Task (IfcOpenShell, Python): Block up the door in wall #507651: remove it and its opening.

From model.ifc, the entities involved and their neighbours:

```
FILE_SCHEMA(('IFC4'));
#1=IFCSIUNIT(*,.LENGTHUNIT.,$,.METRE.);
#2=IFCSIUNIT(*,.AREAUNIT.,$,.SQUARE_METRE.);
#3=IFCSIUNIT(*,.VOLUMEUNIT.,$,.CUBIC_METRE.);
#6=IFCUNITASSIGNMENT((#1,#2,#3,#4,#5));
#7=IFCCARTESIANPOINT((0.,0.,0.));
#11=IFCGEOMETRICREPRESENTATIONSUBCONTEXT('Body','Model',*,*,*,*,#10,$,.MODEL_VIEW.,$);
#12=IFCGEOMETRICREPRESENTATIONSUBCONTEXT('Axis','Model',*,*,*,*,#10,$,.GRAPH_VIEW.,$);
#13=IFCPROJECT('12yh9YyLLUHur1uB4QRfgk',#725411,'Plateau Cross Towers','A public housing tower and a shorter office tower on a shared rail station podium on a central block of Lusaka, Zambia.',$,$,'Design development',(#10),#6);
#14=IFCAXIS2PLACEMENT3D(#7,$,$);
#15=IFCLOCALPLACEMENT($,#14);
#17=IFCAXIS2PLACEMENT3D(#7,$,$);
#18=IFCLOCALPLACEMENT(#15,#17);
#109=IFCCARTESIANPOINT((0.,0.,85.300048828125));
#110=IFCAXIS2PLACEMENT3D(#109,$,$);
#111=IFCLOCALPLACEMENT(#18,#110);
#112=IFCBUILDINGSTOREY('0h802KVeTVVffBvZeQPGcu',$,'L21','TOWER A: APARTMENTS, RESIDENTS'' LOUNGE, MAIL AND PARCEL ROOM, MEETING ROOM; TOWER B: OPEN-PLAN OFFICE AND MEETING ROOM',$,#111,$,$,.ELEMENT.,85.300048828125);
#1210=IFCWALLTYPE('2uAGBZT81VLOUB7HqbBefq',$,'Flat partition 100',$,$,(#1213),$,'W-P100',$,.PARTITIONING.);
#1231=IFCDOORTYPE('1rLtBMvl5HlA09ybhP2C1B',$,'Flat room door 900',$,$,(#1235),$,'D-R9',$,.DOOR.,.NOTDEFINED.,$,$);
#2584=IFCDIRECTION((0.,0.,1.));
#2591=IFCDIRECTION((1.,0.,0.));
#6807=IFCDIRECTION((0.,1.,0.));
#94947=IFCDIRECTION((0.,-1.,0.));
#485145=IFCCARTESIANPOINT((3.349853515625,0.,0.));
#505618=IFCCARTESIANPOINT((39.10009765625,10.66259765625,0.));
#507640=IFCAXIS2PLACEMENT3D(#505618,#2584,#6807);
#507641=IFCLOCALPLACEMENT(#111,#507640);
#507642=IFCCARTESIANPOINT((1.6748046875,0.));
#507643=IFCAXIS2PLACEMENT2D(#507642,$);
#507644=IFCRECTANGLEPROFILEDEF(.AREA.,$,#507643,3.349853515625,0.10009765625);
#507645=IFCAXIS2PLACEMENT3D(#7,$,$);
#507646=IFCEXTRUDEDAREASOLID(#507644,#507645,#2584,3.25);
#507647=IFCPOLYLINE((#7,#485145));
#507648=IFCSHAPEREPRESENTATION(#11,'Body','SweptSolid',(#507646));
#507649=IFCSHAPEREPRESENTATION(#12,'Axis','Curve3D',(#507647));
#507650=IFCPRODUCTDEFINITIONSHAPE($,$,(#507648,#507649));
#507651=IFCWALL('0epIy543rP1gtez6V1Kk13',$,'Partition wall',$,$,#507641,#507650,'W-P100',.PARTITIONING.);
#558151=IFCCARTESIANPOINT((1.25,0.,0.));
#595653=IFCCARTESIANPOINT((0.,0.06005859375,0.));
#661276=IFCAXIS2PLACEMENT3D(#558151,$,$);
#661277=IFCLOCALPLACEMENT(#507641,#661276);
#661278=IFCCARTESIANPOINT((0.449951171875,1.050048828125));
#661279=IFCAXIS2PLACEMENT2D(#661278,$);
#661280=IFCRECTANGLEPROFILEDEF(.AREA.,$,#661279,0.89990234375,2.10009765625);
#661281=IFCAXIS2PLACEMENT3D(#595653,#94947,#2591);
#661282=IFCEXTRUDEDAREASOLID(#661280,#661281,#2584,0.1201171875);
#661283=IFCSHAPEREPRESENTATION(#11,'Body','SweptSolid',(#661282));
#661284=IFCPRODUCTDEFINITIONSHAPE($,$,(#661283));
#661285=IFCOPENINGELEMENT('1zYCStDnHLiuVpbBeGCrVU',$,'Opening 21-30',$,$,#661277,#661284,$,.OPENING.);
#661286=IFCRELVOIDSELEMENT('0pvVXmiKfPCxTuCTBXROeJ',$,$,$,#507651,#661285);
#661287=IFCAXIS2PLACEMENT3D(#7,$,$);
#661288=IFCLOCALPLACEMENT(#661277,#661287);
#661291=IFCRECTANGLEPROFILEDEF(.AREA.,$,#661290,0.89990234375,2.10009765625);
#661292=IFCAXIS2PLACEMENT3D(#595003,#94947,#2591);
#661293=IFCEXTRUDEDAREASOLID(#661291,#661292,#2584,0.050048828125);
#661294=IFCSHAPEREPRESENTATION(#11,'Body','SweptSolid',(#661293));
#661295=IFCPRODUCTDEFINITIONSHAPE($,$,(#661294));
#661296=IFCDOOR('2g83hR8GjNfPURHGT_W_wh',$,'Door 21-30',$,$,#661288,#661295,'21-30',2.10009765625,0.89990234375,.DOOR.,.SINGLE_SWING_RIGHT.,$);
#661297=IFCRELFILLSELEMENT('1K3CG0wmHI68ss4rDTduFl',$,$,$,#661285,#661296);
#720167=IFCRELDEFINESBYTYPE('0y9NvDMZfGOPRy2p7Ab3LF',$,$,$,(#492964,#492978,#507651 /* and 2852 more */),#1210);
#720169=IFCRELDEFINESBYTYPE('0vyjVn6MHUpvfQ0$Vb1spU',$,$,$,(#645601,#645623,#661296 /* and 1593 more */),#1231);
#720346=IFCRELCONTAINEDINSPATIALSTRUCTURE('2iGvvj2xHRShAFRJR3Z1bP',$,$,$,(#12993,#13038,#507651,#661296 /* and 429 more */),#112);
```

```python
import ifcopenshell
import ifcopenshell.api.feature
import ifcopenshell.api.root
import ifcopenshell.geom
import ifcopenshell.util.shape

model = ifcopenshell.open("model.ifc")
settings = ifcopenshell.geom.settings()


def volume(element):
    """Net volume in cubic metres, openings subtracted."""
    shape = ifcopenshell.geom.create_shape(settings, element)
    return ifcopenshell.util.shape.get_volume(shape.geometry)


door = model.by_guid("2g83hR8GjNfPURHGT_W_wh")
opening = door.FillsVoids[0].RelatingOpeningElement
wall = opening.VoidsElements[0].RelatingBuildingElement
before = volume(wall)

ifcopenshell.api.root.remove_product(model, product=door)
ifcopenshell.api.feature.remove_feature(model, feature=opening)

after = volume(wall)

print(f"wall volume {before:.3f} -> {after:.3f} m3")

model.write("model_rev.ifc")
```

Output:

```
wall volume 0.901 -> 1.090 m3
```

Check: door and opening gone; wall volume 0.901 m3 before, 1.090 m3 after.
